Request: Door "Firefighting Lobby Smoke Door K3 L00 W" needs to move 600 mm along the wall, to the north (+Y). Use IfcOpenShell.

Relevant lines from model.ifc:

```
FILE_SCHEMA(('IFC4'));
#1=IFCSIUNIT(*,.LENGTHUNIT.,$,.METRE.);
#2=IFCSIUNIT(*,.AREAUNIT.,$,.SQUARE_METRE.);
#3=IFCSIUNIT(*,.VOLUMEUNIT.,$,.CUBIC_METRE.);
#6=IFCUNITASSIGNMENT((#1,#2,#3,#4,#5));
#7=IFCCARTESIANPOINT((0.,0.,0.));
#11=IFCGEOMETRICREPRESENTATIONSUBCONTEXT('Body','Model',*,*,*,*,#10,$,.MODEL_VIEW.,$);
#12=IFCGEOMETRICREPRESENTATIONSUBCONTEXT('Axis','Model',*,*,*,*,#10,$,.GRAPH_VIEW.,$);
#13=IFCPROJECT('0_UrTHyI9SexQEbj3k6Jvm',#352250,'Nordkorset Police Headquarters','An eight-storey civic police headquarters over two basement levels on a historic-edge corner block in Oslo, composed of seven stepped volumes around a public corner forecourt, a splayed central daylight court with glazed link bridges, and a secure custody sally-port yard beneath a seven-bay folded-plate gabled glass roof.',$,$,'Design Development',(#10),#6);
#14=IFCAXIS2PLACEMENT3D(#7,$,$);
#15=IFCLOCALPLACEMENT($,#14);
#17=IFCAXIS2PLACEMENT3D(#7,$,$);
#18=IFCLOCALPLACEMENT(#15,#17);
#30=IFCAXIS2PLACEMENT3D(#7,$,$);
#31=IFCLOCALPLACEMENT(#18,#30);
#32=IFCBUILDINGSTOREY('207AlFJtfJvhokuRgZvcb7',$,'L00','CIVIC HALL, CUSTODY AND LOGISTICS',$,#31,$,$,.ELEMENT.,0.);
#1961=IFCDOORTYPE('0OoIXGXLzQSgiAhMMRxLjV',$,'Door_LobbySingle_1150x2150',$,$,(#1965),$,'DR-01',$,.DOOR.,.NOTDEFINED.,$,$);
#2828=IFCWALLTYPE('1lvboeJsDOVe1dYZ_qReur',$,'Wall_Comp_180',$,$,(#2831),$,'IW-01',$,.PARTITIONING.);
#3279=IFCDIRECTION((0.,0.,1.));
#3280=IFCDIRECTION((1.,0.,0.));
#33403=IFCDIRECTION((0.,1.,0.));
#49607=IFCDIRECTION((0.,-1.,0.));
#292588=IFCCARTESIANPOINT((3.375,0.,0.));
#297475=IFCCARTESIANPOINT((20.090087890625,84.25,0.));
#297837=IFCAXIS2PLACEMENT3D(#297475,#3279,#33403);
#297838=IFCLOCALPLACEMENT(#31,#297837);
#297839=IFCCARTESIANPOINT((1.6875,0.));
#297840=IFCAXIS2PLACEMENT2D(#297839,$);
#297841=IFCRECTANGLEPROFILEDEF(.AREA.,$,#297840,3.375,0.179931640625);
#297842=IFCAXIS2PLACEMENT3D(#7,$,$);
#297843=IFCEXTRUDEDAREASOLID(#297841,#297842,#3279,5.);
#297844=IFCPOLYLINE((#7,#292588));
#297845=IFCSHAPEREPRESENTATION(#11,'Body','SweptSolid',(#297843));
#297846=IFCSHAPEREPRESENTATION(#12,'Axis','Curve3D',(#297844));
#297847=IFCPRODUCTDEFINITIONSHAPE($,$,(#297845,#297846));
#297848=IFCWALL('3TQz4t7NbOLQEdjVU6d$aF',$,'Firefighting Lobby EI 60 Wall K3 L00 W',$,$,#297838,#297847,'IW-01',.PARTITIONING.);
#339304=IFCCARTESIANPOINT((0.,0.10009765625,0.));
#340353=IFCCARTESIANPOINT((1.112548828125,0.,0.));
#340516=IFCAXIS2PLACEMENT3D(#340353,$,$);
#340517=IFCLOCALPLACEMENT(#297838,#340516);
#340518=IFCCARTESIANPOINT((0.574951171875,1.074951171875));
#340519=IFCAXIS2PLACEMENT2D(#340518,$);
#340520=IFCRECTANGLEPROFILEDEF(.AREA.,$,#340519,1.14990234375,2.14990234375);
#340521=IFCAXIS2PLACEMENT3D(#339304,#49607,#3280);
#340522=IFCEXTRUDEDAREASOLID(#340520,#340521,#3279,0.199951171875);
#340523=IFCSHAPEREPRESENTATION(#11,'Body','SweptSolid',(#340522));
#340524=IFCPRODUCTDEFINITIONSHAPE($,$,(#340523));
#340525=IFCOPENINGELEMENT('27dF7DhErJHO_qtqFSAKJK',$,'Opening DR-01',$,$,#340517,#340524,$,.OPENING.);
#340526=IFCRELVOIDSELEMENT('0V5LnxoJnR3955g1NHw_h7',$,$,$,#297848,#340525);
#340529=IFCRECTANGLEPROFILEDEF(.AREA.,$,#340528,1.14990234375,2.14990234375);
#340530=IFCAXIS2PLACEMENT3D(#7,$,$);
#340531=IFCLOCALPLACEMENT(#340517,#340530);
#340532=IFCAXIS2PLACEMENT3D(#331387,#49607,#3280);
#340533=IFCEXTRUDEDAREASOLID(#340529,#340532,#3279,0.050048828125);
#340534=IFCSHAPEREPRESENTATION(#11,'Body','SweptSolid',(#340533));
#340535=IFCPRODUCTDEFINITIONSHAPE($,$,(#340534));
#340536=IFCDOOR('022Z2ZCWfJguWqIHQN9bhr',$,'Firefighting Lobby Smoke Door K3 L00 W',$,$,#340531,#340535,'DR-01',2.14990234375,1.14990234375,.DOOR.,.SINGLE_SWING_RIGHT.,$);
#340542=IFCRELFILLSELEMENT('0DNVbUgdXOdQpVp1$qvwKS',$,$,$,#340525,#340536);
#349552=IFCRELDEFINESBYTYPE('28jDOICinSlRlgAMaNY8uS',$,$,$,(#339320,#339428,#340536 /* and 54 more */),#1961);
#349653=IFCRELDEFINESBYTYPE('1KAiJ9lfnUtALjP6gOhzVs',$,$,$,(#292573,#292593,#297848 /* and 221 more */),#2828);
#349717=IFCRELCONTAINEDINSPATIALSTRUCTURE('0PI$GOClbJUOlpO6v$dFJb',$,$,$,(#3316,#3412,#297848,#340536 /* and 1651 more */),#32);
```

```python
import ifcopenshell
import ifcopenshell.api.geometry
import ifcopenshell.util.placement
import ifcopenshell.util.unit

model = ifcopenshell.open("model.ifc")
unit_scale = ifcopenshell.util.unit.calculate_unit_scale(model)

door = model.by_guid("022Z2ZCWfJguWqIHQN9bhr")
opening = door.FillsVoids[0].RelatingOpeningElement
wall = opening.VoidsElements[0].RelatingBuildingElement

wall_matrix = ifcopenshell.util.placement.get_local_placement(wall.ObjectPlacement)
shift = wall_matrix[:3, 0] * 0.6 / unit_scale
before = ifcopenshell.util.placement.get_local_placement(door.ObjectPlacement)[:3, 3].copy()

# The door is placed relative to its opening, so it follows when the opening moves.
matrix = ifcopenshell.util.placement.get_local_placement(opening.ObjectPlacement)
matrix[:3, 3] += shift
ifcopenshell.api.geometry.edit_object_placement(
    model, product=opening, matrix=matrix, is_si=False, should_transform_children=True
)

after = ifcopenshell.util.placement.get_local_placement(door.ObjectPlacement)[:3, 3]
print("door moved by", (after - before).round(3) + 0.0)

model.write("model_v2.ifc")
```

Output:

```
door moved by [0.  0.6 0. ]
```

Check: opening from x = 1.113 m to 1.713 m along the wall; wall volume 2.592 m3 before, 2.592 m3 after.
